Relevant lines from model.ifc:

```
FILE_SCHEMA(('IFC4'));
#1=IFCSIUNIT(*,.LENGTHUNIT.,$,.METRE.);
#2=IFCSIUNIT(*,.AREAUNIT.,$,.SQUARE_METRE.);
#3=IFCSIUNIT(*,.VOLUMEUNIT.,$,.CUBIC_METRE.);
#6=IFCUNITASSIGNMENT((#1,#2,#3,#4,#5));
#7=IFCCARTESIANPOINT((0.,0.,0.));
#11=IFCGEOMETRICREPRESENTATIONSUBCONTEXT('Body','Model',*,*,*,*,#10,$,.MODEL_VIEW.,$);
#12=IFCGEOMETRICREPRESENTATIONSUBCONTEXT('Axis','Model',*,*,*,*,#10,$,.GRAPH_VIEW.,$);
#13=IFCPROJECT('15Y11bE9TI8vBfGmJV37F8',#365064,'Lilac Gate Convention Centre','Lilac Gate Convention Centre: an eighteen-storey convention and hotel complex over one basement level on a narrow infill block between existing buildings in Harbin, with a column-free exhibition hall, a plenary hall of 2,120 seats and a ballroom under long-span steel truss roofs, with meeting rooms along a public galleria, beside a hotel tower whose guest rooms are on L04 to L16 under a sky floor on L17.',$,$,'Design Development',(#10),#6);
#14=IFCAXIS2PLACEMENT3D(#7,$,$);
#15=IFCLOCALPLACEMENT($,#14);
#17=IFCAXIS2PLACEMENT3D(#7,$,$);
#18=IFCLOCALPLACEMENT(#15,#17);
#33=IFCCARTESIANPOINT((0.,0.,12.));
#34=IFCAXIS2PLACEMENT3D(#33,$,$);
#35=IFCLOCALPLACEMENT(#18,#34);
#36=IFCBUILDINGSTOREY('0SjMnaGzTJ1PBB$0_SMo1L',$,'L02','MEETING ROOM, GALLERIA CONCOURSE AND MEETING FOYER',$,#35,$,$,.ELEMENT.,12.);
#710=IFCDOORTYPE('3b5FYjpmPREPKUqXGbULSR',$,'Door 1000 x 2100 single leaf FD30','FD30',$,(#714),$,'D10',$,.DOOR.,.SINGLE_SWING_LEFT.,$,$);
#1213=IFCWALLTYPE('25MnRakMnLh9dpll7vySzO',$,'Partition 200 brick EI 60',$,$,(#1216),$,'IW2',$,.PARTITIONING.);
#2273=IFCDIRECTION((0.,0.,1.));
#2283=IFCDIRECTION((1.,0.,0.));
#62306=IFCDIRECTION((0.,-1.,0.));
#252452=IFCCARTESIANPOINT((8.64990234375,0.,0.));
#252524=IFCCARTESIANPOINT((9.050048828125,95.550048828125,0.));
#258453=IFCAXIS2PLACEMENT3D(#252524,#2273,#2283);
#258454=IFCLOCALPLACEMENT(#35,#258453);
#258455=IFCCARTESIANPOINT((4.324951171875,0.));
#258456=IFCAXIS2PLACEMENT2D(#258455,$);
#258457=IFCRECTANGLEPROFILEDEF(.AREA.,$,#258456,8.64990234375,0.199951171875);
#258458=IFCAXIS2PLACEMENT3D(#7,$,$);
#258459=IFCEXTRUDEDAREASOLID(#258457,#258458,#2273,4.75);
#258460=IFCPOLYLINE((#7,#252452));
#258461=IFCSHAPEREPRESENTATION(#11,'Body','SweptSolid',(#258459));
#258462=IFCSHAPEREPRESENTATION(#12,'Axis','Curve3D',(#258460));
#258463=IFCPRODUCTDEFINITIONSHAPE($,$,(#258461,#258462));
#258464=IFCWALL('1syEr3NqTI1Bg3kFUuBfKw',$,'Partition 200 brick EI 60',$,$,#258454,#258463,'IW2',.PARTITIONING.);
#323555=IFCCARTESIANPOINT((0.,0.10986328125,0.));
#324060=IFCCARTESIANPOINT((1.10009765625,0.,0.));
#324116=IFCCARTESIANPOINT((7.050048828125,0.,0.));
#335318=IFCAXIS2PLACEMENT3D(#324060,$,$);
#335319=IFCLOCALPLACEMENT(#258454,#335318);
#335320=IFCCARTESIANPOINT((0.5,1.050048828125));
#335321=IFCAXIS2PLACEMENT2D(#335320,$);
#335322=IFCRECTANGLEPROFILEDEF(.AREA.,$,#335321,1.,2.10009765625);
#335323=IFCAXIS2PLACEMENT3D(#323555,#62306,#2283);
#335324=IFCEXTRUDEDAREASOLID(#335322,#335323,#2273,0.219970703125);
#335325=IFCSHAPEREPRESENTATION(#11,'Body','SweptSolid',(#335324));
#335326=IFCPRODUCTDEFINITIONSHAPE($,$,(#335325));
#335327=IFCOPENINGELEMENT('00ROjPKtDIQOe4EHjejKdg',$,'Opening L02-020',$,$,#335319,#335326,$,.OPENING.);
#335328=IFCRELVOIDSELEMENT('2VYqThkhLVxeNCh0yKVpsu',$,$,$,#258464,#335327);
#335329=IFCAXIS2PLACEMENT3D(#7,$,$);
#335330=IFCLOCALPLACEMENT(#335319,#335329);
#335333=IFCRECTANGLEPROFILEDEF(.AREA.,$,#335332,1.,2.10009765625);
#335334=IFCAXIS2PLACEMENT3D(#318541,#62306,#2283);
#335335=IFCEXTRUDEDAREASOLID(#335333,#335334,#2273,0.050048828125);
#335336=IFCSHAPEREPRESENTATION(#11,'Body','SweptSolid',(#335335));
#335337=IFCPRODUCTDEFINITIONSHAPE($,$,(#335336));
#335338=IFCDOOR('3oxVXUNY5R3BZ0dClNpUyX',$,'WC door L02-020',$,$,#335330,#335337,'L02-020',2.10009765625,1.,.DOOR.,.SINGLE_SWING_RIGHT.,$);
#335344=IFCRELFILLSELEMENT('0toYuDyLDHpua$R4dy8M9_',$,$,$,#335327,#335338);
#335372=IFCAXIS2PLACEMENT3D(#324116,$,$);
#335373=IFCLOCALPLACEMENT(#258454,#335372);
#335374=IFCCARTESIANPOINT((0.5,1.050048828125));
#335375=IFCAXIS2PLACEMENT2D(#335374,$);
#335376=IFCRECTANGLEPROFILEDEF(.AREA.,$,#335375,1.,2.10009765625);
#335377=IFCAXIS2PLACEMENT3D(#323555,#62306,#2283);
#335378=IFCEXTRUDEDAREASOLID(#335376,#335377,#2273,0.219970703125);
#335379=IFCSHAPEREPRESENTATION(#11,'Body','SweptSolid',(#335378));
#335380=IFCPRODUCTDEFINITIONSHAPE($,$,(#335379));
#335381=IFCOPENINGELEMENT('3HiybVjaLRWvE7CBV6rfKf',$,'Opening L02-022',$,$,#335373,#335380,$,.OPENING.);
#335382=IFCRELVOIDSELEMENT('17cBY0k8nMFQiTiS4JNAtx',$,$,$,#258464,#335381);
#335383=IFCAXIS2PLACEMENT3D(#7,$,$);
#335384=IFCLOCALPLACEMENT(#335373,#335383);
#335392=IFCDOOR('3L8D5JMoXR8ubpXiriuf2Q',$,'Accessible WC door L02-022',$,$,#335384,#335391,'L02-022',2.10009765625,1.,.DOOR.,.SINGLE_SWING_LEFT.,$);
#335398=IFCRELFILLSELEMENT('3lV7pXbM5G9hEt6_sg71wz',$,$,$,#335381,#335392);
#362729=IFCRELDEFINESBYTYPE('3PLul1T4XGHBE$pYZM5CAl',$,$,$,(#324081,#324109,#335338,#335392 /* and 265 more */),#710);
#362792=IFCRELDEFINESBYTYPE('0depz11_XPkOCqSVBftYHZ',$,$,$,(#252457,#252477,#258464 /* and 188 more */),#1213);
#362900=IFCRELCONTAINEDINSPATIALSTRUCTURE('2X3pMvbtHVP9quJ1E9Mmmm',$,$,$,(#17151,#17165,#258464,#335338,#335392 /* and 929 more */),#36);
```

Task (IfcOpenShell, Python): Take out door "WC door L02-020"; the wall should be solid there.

```python
import ifcopenshell
import ifcopenshell.api.feature
import ifcopenshell.api.root
import ifcopenshell.geom
import ifcopenshell.util.shape

model = ifcopenshell.open("model.ifc")
settings = ifcopenshell.geom.settings()


def volume(element):
    """Net volume in cubic metres, openings subtracted."""
    shape = ifcopenshell.geom.create_shape(settings, element)
    return ifcopenshell.util.shape.get_volume(shape.geometry)


door = model.by_guid("3oxVXUNY5R3BZ0dClNpUyX")
opening = door.FillsVoids[0].RelatingOpeningElement
wall = opening.VoidsElements[0].RelatingBuildingElement
before = volume(wall)

ifcopenshell.api.root.remove_product(model, product=door)
ifcopenshell.api.feature.remove_feature(model, feature=opening)

after = volume(wall)

print(f"wall volume {before:.3f} -> {after:.3f} m3")

model.write("model-out.ifc")
```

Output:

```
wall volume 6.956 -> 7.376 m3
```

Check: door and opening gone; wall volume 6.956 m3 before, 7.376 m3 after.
